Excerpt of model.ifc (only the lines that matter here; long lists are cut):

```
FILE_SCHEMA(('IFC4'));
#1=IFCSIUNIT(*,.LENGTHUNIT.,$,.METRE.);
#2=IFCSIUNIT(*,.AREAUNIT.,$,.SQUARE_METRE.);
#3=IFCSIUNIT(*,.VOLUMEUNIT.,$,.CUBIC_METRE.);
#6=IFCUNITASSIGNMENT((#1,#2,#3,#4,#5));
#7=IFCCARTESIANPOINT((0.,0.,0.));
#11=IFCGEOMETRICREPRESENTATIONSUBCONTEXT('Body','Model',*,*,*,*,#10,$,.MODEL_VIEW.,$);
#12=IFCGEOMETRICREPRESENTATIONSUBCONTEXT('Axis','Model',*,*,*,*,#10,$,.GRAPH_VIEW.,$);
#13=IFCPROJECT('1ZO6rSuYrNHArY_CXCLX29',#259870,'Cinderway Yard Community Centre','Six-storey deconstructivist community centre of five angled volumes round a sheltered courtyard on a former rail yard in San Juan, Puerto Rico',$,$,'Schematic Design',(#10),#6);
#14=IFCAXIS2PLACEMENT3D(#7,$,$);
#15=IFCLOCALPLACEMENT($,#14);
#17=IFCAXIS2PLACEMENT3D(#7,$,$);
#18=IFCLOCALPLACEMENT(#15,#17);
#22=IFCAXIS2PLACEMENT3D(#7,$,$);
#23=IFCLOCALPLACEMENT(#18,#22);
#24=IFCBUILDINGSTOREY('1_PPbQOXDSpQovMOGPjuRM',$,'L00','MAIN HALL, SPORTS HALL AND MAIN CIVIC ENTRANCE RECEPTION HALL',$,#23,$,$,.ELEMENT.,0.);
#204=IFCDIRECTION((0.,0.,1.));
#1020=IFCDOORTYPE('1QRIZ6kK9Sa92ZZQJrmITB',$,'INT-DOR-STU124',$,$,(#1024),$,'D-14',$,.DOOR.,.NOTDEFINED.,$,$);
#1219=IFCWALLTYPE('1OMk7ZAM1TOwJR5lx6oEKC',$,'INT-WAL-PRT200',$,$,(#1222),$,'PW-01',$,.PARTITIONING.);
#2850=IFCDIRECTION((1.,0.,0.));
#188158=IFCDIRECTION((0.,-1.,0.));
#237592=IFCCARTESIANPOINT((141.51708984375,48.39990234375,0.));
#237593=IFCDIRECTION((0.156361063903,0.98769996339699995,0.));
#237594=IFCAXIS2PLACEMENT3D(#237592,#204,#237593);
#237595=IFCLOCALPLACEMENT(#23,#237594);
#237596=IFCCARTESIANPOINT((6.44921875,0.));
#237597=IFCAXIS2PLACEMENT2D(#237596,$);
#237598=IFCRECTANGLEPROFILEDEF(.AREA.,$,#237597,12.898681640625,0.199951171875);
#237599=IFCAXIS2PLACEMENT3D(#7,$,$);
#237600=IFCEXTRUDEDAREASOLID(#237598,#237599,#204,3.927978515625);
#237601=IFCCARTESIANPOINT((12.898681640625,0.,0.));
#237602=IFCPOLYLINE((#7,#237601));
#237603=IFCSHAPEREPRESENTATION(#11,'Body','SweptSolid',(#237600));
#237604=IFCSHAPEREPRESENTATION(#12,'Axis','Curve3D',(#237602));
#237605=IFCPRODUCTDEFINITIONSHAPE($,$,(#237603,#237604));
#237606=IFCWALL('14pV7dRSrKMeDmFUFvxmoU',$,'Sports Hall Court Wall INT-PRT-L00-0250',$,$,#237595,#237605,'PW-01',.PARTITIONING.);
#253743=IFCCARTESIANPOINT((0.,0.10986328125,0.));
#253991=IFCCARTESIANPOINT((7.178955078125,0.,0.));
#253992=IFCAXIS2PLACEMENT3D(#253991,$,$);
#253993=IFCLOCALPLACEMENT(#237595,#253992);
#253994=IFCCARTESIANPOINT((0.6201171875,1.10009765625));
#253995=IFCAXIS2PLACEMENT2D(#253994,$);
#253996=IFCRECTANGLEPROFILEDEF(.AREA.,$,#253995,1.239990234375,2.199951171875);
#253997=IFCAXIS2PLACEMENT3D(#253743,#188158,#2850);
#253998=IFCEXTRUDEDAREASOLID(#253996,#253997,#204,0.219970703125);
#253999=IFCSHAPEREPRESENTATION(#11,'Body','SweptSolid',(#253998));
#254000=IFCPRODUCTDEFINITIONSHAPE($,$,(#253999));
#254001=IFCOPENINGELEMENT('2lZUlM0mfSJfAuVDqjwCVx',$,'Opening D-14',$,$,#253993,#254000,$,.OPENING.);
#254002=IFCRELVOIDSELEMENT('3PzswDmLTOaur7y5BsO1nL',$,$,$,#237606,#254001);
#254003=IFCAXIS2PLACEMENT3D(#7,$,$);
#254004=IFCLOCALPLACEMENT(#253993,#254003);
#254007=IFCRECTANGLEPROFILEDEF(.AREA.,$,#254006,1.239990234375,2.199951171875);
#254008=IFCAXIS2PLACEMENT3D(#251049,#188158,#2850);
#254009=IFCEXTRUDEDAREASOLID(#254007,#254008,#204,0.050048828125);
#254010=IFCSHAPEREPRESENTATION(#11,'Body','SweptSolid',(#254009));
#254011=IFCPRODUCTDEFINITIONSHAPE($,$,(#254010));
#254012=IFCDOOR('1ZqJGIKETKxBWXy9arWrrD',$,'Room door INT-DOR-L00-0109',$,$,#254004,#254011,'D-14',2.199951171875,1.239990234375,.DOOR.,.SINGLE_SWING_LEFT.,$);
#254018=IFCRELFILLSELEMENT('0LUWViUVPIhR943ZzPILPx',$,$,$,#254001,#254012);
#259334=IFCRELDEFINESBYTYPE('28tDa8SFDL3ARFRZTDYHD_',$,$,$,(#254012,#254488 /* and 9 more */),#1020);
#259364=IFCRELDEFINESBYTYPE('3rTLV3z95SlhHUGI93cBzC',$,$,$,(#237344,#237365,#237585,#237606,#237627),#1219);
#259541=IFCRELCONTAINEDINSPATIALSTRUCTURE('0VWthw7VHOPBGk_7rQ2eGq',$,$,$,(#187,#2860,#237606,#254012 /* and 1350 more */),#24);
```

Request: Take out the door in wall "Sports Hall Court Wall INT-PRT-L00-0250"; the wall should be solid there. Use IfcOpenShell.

```python
import ifcopenshell
import ifcopenshell.api.feature
import ifcopenshell.api.root
import ifcopenshell.geom
import ifcopenshell.util.shape

model = ifcopenshell.open("model.ifc")
settings = ifcopenshell.geom.settings()


def volume(element):
    """Net volume in cubic metres, openings subtracted."""
    shape = ifcopenshell.geom.create_shape(settings, element)
    return ifcopenshell.util.shape.get_volume(shape.geometry)


door = model.by_guid("1ZqJGIKETKxBWXy9arWrrD")
opening = door.FillsVoids[0].RelatingOpeningElement
wall = opening.VoidsElements[0].RelatingBuildingElement
before = volume(wall)

ifcopenshell.api.root.remove_product(model, product=door)
ifcopenshell.api.feature.remove_feature(model, feature=opening)

after = volume(wall)

print(f"wall volume {before:.3f} -> {after:.3f} m3")

model.write("model_updated.ifc")
```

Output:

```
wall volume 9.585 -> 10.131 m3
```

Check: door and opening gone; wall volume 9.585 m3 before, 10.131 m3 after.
